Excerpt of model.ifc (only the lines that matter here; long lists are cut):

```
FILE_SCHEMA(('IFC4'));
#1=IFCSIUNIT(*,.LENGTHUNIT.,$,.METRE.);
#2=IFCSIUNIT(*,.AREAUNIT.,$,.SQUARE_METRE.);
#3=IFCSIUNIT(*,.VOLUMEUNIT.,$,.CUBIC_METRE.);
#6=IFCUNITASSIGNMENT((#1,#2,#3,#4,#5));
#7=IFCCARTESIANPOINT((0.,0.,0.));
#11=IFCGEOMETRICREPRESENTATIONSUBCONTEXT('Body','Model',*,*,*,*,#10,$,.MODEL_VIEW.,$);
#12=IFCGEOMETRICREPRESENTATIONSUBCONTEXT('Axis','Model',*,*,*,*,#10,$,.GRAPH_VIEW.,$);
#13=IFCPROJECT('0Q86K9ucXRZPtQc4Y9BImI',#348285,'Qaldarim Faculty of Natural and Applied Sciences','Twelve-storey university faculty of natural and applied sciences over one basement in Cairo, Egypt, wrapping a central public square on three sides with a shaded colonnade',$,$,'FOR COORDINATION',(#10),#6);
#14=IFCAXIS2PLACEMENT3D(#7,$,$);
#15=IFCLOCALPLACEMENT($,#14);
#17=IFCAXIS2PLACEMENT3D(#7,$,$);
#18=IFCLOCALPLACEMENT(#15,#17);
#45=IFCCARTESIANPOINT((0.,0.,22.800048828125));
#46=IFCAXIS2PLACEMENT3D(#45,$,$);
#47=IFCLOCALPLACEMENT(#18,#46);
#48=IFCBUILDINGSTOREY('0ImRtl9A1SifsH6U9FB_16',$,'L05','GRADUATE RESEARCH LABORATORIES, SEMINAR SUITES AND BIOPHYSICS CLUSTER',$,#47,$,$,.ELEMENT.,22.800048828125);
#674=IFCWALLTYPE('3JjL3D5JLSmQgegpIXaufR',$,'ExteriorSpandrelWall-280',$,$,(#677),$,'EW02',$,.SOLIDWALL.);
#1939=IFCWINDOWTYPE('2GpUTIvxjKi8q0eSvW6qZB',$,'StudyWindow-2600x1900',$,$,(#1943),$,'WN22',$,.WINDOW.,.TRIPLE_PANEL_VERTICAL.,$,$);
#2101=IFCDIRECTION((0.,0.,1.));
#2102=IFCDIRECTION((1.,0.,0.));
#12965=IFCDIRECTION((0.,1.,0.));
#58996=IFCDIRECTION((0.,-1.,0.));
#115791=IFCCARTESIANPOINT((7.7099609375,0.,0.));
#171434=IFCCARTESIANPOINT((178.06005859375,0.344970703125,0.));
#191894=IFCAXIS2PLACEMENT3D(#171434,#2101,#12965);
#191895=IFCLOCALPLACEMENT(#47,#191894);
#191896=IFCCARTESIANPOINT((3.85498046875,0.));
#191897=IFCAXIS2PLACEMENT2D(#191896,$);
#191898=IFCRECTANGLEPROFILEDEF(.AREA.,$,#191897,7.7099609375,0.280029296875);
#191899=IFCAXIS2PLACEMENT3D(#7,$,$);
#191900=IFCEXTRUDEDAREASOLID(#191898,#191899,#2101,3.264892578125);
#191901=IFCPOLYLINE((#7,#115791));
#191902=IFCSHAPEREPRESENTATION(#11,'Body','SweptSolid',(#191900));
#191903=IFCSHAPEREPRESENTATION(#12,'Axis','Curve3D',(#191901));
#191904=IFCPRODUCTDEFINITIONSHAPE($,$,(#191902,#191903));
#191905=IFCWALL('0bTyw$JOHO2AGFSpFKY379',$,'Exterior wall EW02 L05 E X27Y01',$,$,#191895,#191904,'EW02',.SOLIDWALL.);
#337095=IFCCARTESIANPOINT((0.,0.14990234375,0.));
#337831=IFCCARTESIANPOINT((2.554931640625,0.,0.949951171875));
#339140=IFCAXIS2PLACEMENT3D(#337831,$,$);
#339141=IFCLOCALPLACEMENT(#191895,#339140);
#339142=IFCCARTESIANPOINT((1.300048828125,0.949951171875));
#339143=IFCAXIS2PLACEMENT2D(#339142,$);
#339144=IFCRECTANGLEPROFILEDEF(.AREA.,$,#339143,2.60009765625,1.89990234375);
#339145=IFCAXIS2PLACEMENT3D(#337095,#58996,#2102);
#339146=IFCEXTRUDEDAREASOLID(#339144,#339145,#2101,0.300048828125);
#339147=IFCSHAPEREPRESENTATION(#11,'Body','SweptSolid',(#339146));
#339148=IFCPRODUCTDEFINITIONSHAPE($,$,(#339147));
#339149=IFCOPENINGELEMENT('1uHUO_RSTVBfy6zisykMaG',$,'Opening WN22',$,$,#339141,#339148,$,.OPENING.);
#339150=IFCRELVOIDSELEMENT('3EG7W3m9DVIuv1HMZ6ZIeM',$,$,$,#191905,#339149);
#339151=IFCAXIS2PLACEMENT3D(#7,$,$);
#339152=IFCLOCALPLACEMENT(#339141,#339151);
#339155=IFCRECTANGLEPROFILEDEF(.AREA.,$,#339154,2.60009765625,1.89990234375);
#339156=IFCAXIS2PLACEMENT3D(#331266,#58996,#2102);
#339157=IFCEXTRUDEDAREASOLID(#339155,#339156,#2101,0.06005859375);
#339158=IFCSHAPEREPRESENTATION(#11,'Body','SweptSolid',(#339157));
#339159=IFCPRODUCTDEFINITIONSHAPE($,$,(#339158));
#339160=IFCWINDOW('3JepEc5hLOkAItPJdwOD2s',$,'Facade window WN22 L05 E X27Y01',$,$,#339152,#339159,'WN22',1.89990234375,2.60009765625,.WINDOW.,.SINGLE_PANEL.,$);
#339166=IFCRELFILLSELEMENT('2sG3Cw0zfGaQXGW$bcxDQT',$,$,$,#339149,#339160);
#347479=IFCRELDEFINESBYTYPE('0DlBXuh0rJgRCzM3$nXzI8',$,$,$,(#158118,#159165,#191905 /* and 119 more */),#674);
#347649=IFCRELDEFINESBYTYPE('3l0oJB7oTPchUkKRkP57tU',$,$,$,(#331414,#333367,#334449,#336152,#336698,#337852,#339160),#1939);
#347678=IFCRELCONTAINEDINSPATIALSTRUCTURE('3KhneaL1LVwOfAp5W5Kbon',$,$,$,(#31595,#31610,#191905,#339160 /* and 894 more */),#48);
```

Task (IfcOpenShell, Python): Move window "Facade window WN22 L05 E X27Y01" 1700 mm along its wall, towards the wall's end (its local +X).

```python
import ifcopenshell
import ifcopenshell.api.geometry
import ifcopenshell.util.placement

model = ifcopenshell.open("model.ifc")

window = model.by_guid("3JepEc5hLOkAItPJdwOD2s")
opening = window.FillsVoids[0].RelatingOpeningElement
wall = opening.VoidsElements[0].RelatingBuildingElement

wall_matrix = ifcopenshell.util.placement.get_local_placement(wall.ObjectPlacement)
shift = wall_matrix[:3, 0] * 1.7
before = ifcopenshell.util.placement.get_local_placement(window.ObjectPlacement)[:3, 3].copy()

# The window is placed relative to its opening, so it follows when the opening moves.
matrix = ifcopenshell.util.placement.get_local_placement(opening.ObjectPlacement)
matrix[:3, 3] += shift
ifcopenshell.api.geometry.edit_object_placement(
    model, product=opening, matrix=matrix, is_si=False, should_transform_children=True
)

after = ifcopenshell.util.placement.get_local_placement(window.ObjectPlacement)[:3, 3]
print("window moved by", (after - before).round(3) + 0.0)

model.write("model-out.ifc")
```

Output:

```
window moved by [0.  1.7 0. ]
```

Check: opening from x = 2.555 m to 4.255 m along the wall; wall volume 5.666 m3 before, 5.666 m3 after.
